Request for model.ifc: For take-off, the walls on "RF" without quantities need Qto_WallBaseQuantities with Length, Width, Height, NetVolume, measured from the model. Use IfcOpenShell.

First a look at what the model holds.

```python
import ifcopenshell
import ifcopenshell.util.element
import ifcopenshell.util.unit

model = ifcopenshell.open("model.ifc")
print(model.schema)
for unit_type in ("LENGTHUNIT", "AREAUNIT", "VOLUMEUNIT"):
    print(unit_type, ifcopenshell.util.unit.calculate_unit_scale(model, unit_type))
storey = next(s for s in model.by_type("IfcBuildingStorey") if s.Name == "RF")
walls = [e for e in ifcopenshell.util.element.get_decomposition(storey) if e.is_a("IfcWall")]
for e in sorted(walls, key=lambda e: e.id()):
    print(e.id(), e.is_a(), e.Name, list(ifcopenshell.util.element.get_psets(e, qtos_only=True)), sep=" | ")
```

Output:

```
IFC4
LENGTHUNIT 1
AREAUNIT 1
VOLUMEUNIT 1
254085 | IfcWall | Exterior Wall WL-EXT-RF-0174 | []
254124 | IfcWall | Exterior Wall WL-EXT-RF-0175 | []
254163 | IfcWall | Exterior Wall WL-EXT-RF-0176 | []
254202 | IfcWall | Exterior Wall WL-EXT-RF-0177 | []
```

```python
import ifcopenshell
import ifcopenshell.api.pset
import ifcopenshell.geom
import ifcopenshell.util.element
import ifcopenshell.util.shape
import ifcopenshell.util.unit

model = ifcopenshell.open("model.ifc")
unit_scale = ifcopenshell.util.unit.calculate_unit_scale(model)
volume_scale = ifcopenshell.util.unit.calculate_unit_scale(model, "VOLUMEUNIT")
settings = ifcopenshell.geom.settings()

storey = next(s for s in model.by_type("IfcBuildingStorey") if s.Name == "RF")
walls = [e for e in ifcopenshell.util.element.get_decomposition(storey) if e.is_a("IfcWall")]

for e in sorted(walls, key=lambda e: e.id()):
    if ifcopenshell.util.element.get_psets(e, qtos_only=True, should_inherit=False):
        continue
    # Geometry comes back in metres, in the element's own axes.
    shape = ifcopenshell.geom.create_shape(settings, e)
    values = {
        "Length": ifcopenshell.util.shape.get_x(shape.geometry) / unit_scale,
        "Width": ifcopenshell.util.shape.get_y(shape.geometry) / unit_scale,
        "Height": ifcopenshell.util.shape.get_z(shape.geometry) / unit_scale,
        "NetVolume": ifcopenshell.util.shape.get_volume(shape.geometry) / volume_scale,
    }
    qto = ifcopenshell.api.pset.add_qto(model, product=e, name="Qto_WallBaseQuantities")
    ifcopenshell.api.pset.edit_qto(model, qto=qto, properties=values)
    print(e.id(), {k: round(v, 3) for k, v in values.items()})

model.write("model_v2.ifc")
```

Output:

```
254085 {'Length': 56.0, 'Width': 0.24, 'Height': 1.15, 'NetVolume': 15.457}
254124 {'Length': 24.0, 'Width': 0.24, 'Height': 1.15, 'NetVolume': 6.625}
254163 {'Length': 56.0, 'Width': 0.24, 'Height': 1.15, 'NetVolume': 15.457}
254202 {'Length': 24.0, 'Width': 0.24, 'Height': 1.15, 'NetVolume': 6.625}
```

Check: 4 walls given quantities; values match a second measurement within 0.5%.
